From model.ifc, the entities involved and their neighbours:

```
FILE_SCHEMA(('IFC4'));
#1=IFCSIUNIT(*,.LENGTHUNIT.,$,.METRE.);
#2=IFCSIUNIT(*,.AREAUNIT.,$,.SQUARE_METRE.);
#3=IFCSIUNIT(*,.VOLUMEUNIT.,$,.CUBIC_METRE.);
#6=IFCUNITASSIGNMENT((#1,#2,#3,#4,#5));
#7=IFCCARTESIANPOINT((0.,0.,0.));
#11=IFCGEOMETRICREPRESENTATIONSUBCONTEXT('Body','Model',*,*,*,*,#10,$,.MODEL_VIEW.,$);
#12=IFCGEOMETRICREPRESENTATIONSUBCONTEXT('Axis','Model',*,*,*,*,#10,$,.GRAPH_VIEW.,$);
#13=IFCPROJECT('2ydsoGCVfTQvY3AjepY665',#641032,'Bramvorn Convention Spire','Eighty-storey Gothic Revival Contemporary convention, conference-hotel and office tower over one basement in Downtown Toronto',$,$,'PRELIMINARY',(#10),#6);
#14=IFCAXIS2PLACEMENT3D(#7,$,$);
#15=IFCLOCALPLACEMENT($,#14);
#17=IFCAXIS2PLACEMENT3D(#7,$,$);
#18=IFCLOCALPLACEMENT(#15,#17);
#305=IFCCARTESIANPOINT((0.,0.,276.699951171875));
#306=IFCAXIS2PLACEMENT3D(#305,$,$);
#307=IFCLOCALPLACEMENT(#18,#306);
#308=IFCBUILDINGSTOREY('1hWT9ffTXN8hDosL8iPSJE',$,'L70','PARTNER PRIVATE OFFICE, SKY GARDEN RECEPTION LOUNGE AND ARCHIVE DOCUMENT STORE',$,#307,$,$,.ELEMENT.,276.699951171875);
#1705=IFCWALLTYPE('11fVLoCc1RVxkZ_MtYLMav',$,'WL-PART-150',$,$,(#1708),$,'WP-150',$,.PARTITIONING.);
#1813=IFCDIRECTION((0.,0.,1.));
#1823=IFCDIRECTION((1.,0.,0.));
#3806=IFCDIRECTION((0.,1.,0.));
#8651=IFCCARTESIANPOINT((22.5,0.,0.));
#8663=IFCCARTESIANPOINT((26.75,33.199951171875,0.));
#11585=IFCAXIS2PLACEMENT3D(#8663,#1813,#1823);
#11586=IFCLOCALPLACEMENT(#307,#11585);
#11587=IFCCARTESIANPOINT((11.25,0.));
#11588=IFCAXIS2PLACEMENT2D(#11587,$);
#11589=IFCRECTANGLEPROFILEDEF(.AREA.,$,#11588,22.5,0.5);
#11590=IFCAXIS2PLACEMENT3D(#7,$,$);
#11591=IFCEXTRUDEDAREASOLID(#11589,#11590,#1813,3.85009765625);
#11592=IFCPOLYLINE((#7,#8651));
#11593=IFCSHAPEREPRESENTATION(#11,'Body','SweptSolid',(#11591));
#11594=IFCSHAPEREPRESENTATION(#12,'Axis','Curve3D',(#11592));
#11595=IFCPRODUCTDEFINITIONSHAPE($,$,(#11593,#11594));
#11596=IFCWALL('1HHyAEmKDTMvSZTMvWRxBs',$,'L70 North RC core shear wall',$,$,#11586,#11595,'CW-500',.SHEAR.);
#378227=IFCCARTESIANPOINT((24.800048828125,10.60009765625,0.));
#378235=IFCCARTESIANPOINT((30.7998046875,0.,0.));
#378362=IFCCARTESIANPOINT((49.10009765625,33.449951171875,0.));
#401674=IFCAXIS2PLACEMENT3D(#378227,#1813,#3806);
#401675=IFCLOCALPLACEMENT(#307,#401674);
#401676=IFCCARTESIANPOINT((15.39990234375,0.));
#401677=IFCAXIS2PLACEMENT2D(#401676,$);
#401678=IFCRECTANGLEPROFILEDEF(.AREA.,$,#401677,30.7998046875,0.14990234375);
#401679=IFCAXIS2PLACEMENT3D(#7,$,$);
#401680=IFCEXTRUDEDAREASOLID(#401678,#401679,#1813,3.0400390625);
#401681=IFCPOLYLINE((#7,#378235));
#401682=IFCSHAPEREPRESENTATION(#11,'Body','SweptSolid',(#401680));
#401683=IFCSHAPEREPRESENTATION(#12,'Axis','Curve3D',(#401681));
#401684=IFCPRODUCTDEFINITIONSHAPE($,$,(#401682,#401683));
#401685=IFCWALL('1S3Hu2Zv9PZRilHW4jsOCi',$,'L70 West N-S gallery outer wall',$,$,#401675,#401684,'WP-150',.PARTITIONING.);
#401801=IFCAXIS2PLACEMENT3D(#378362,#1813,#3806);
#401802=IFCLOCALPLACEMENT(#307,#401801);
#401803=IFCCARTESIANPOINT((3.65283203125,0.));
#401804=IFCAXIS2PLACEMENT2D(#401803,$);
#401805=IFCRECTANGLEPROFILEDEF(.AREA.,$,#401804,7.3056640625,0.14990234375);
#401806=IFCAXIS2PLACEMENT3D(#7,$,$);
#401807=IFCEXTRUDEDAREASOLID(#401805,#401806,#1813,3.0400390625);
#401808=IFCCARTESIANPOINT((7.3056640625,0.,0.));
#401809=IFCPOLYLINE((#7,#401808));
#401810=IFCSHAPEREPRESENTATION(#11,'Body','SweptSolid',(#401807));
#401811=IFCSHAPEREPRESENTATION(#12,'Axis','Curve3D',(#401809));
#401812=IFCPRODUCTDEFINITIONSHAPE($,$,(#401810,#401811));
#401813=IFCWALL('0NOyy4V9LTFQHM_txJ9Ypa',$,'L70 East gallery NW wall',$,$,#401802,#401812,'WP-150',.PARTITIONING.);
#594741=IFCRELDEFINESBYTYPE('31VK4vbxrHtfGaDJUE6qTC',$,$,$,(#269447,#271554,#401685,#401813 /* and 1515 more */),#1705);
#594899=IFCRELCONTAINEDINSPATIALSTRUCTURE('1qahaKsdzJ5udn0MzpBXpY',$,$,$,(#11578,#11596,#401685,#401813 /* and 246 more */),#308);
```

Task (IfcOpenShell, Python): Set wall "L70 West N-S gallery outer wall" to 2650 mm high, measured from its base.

```python
import ifcopenshell
import ifcopenshell.geom
import ifcopenshell.util.representation
import ifcopenshell.util.shape

model = ifcopenshell.open("model.ifc")
settings = ifcopenshell.geom.settings()


def volume(element):
    """Net volume in cubic metres, openings subtracted."""
    shape = ifcopenshell.geom.create_shape(settings, element)
    return ifcopenshell.util.shape.get_volume(shape.geometry)


wall = model.by_guid("1S3Hu2Zv9PZRilHW4jsOCi")
before = volume(wall)

body = ifcopenshell.util.representation.get_representation(wall, "Model", "Body")
solid = body.Items[0]
old_height = solid.Depth
solid.Depth = 2.65
after = volume(wall)

print(f"height {old_height:g} -> {solid.Depth:g}, volume {before:.3f} -> {after:.3f} m3")

model.write("model_rev.ifc")
```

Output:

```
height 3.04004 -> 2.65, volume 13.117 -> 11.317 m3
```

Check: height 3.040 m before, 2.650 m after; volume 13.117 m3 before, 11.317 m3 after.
